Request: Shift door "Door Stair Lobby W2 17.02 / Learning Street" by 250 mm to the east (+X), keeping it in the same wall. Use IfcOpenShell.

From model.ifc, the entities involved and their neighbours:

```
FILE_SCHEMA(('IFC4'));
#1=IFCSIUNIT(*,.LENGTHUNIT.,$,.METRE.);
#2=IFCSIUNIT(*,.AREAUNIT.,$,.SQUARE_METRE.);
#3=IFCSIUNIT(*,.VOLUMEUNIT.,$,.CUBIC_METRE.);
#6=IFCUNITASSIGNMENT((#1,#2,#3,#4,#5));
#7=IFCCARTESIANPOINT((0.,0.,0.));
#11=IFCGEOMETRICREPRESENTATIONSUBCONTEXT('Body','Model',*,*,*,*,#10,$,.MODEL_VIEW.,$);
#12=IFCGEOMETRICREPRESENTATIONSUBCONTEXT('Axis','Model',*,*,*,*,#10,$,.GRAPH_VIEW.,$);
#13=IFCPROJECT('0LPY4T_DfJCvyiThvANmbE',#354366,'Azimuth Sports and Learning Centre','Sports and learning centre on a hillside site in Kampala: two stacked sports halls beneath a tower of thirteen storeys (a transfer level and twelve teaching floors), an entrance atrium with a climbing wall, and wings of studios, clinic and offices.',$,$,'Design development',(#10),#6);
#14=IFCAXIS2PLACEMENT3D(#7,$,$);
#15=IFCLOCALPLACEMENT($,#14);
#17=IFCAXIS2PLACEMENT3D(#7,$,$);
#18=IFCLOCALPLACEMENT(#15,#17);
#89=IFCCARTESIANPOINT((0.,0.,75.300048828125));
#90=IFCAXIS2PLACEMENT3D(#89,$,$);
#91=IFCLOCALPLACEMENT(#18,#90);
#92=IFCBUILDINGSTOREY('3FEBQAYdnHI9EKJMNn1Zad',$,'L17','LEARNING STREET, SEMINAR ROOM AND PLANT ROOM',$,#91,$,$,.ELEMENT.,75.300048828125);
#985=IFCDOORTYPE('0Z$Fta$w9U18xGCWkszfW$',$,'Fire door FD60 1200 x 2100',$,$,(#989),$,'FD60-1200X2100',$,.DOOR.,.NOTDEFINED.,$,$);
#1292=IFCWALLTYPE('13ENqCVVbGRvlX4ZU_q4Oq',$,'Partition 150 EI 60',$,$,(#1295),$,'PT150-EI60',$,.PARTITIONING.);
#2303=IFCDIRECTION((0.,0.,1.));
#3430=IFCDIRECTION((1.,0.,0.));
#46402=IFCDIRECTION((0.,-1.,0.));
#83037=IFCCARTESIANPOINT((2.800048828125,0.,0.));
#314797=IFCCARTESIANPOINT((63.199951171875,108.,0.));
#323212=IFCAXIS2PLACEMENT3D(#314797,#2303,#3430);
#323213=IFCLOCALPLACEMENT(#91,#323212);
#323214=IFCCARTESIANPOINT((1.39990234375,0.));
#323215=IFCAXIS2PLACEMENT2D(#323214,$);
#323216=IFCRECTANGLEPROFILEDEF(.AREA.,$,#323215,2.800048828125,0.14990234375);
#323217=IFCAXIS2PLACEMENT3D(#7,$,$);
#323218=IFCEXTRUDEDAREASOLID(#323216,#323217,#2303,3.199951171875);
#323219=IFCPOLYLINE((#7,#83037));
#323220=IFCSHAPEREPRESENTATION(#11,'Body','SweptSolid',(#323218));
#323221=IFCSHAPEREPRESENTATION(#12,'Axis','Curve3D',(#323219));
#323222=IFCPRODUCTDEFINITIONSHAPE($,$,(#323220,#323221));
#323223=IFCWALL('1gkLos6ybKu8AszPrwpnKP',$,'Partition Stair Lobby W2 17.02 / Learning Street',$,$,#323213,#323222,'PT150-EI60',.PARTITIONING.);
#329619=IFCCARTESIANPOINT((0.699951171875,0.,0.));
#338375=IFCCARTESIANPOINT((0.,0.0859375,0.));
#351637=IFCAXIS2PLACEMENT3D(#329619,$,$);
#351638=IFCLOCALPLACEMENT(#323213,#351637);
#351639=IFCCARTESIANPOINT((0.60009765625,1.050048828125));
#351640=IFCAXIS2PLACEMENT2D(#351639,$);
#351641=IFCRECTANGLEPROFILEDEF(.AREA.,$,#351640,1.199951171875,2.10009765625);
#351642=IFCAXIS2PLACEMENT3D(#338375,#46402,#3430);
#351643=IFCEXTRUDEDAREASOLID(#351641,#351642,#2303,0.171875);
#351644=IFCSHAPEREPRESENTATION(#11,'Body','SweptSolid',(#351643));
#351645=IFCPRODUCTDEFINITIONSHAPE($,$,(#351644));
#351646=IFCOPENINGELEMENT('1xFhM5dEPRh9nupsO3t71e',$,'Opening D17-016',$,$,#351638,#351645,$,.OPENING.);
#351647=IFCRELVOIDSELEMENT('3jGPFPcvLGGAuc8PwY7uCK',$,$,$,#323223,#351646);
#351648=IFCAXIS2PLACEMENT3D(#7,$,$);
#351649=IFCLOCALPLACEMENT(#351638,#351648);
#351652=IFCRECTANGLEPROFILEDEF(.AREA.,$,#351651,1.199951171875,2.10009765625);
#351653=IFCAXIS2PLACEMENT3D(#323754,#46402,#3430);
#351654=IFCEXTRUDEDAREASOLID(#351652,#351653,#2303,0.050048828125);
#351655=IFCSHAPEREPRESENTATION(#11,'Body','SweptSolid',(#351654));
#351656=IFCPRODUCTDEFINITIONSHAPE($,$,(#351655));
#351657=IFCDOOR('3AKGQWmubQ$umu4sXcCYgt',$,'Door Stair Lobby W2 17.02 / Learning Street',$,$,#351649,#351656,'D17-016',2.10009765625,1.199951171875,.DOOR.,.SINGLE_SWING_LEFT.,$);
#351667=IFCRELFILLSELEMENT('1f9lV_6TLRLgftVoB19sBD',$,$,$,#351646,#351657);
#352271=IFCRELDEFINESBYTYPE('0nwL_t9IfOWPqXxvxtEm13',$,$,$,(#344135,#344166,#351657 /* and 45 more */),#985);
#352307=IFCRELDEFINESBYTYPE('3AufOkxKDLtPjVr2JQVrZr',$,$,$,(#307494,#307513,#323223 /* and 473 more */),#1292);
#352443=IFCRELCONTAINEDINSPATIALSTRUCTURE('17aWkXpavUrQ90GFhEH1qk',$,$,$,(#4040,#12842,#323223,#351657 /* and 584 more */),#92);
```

```python
import ifcopenshell
import ifcopenshell.api.geometry
import ifcopenshell.util.placement
import ifcopenshell.util.unit

model = ifcopenshell.open("model.ifc")
unit_scale = ifcopenshell.util.unit.calculate_unit_scale(model)

door = model.by_guid("3AKGQWmubQ$umu4sXcCYgt")
opening = door.FillsVoids[0].RelatingOpeningElement
wall = opening.VoidsElements[0].RelatingBuildingElement

wall_matrix = ifcopenshell.util.placement.get_local_placement(wall.ObjectPlacement)
shift = wall_matrix[:3, 0] * 0.25 / unit_scale
before = ifcopenshell.util.placement.get_local_placement(door.ObjectPlacement)[:3, 3].copy()

# The door is placed relative to its opening, so it follows when the opening moves.
matrix = ifcopenshell.util.placement.get_local_placement(opening.ObjectPlacement)
matrix[:3, 3] += shift
ifcopenshell.api.geometry.edit_object_placement(
    model, product=opening, matrix=matrix, is_si=False, should_transform_children=True
)

after = ifcopenshell.util.placement.get_local_placement(door.ObjectPlacement)[:3, 3]
print("door moved by", (after - before).round(3) + 0.0)

model.write("model-out.ifc")
```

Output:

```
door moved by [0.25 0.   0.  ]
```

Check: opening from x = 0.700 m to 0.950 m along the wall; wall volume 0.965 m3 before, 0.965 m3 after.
